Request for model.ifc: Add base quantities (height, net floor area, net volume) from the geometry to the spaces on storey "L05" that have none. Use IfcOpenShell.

First a look at what the model holds.

```python
import ifcopenshell
import ifcopenshell.util.element
import ifcopenshell.util.unit

model = ifcopenshell.open("model.ifc")
print(model.schema)
for unit_type in ("LENGTHUNIT", "AREAUNIT", "VOLUMEUNIT"):
    print(unit_type, ifcopenshell.util.unit.calculate_unit_scale(model, unit_type))
storey = next(s for s in model.by_type("IfcBuildingStorey") if s.Name == "L05")
spaces = [e for e in ifcopenshell.util.element.get_decomposition(storey) if e.is_a("IfcSpace")]
for e in sorted(spaces, key=lambda e: e.id()):
    print(e.id(), e.is_a(), e.Name, list(ifcopenshell.util.element.get_psets(e, qtos_only=True)), sep=" | ")
```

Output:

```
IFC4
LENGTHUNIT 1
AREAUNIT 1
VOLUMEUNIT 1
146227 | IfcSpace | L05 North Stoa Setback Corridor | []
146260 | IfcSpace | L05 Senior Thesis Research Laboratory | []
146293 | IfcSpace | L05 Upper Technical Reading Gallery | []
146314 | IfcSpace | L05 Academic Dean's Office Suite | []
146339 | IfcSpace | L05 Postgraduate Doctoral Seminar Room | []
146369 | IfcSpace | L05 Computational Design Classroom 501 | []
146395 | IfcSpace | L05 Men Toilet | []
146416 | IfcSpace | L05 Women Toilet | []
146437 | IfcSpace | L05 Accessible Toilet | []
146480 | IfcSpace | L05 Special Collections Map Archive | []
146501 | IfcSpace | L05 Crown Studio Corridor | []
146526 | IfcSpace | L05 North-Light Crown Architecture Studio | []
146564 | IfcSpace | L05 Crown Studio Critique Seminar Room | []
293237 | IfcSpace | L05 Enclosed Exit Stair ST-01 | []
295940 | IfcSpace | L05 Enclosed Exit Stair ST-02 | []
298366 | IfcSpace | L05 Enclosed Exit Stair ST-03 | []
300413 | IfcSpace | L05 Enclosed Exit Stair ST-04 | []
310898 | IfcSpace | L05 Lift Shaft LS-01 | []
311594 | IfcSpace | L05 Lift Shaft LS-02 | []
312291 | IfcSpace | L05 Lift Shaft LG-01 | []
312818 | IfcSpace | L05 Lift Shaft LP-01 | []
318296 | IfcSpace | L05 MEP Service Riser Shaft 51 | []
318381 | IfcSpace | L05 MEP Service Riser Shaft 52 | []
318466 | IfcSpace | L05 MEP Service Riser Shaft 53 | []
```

```python
import ifcopenshell
import ifcopenshell.api.pset
import ifcopenshell.geom
import ifcopenshell.util.element
import ifcopenshell.util.shape
import ifcopenshell.util.unit

model = ifcopenshell.open("model.ifc")
unit_scale = ifcopenshell.util.unit.calculate_unit_scale(model)
area_scale = ifcopenshell.util.unit.calculate_unit_scale(model, "AREAUNIT")
volume_scale = ifcopenshell.util.unit.calculate_unit_scale(model, "VOLUMEUNIT")
settings = ifcopenshell.geom.settings()

storey = next(s for s in model.by_type("IfcBuildingStorey") if s.Name == "L05")
spaces = [e for e in ifcopenshell.util.element.get_decomposition(storey) if e.is_a("IfcSpace")]

for e in sorted(spaces, key=lambda e: e.id()):
    if ifcopenshell.util.element.get_psets(e, qtos_only=True, should_inherit=False):
        continue
    # Geometry comes back in metres, in the element's own axes.
    shape = ifcopenshell.geom.create_shape(settings, e)
    values = {
        "Height": ifcopenshell.util.shape.get_z(shape.geometry) / unit_scale,
        "NetFloorArea": ifcopenshell.util.shape.get_footprint_area(shape.geometry) / area_scale,
        "NetVolume": ifcopenshell.util.shape.get_volume(shape.geometry) / volume_scale,
    }
    qto = ifcopenshell.api.pset.add_qto(model, product=e, name="Qto_SpaceBaseQuantities")
    ifcopenshell.api.pset.edit_qto(model, qto=qto, properties=values)
    print(e.id(), {k: round(v, 3) for k, v in values.items()})

model.write("model_edited.ifc")
```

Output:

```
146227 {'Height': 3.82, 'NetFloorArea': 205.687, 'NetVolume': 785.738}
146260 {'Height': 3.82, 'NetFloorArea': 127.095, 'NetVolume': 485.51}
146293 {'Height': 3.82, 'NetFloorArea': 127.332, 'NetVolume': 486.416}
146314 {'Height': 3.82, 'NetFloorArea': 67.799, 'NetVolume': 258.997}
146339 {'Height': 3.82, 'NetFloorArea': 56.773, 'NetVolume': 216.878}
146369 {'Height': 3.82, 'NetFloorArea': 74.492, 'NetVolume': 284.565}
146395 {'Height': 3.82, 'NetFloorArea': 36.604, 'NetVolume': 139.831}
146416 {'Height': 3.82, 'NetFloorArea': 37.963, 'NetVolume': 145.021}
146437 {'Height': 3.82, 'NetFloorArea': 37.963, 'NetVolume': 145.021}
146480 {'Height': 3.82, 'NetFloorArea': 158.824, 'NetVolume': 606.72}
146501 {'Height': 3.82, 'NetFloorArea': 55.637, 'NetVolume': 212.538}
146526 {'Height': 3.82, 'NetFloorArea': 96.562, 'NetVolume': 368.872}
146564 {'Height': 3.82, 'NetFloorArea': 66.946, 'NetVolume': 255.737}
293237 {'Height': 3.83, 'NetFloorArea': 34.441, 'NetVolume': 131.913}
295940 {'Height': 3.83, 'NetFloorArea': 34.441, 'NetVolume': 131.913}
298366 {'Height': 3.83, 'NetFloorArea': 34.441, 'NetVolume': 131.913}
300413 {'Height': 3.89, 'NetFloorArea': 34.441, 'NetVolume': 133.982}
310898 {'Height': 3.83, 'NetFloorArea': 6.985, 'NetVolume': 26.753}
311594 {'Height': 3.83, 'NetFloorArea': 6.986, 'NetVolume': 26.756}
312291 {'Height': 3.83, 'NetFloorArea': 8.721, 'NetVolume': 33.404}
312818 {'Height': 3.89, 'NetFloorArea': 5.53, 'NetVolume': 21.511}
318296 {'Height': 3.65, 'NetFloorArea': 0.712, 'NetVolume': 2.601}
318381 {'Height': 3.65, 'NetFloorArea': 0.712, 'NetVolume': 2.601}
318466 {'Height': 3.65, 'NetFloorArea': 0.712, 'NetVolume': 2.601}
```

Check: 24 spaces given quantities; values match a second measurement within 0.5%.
